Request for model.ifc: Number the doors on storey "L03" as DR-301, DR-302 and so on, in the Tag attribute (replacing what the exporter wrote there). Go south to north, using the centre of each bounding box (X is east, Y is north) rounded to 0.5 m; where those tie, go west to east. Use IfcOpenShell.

First a look at what the model holds.

```python
import ifcopenshell
import ifcopenshell.util.element
import ifcopenshell.util.placement

model = ifcopenshell.open("model.ifc")
print(model.schema)
storey = next(s for s in model.by_type("IfcBuildingStorey") if s.Name == "L03")
doors = [e for e in ifcopenshell.util.element.get_decomposition(storey) if e.is_a("IfcDoor")]
for e in sorted(doors, key=lambda e: e.id()):
    origin = ifcopenshell.util.placement.get_local_placement(e.ObjectPlacement)[:3, 3]
    print(e.id(), e.Tag, e.Name, origin.round(2) + 0.0, sep=" | ")
```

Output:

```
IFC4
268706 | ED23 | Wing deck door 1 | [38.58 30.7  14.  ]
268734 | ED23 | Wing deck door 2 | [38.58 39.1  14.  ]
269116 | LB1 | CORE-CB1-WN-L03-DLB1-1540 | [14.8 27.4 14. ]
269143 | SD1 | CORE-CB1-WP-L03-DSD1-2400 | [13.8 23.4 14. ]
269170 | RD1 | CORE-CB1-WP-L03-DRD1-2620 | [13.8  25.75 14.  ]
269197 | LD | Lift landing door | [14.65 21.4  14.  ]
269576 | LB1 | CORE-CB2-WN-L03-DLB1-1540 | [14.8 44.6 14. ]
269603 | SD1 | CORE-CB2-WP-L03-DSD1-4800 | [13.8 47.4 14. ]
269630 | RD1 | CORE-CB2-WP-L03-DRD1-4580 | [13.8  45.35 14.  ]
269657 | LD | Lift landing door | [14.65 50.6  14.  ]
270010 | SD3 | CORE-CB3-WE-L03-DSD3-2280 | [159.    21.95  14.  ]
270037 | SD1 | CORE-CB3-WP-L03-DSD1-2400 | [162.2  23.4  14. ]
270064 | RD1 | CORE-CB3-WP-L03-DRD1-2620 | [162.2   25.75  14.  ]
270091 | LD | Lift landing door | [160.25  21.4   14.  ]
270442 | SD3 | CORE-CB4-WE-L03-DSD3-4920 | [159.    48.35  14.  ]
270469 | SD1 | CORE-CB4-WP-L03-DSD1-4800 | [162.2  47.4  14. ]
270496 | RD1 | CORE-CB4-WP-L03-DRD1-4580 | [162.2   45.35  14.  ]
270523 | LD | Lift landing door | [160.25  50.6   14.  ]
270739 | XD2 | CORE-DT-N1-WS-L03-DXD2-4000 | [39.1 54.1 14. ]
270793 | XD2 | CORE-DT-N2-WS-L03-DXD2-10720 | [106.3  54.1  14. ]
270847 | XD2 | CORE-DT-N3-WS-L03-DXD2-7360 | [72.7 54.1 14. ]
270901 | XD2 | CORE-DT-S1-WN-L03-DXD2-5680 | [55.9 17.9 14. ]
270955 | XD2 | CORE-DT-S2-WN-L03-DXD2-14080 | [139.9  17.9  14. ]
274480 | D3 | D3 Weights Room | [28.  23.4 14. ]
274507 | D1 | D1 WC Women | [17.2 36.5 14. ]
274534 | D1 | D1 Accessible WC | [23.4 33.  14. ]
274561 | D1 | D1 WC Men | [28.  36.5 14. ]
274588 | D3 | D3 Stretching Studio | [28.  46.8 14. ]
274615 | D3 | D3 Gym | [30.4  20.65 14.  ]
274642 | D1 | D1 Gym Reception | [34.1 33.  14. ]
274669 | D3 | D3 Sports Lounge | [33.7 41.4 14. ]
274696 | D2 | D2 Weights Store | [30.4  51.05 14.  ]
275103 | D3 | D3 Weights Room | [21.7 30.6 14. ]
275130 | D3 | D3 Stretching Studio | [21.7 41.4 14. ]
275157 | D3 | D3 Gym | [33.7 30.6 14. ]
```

```python
import ifcopenshell
import ifcopenshell.geom
import ifcopenshell.util.element
import ifcopenshell.util.shape

model = ifcopenshell.open("model.ifc")
settings = ifcopenshell.geom.settings()
settings.set("use-world-coords", True)


def centre(element):
    shape = ifcopenshell.geom.create_shape(settings, element)
    return ifcopenshell.util.shape.get_bbox_centroid(shape.geometry)


storey = next(s for s in model.by_type("IfcBuildingStorey") if s.Name == "L03")
doors = [e for e in ifcopenshell.util.element.get_decomposition(storey) if e.is_a("IfcDoor")]

# Insertion points can sit at a corner or the storey origin, so sort by the geometry (in metres).
centres = {e: centre(e) for e in doors}
doors.sort(key=lambda e: (round(centres[e][1] / 0.5), centres[e][0]))

for i, e in enumerate(doors, start=1):
    number = f"DR-3{i:02d}"
    e.Tag = number
    print(e.id(), number)

model.write("model_updated.ifc")
```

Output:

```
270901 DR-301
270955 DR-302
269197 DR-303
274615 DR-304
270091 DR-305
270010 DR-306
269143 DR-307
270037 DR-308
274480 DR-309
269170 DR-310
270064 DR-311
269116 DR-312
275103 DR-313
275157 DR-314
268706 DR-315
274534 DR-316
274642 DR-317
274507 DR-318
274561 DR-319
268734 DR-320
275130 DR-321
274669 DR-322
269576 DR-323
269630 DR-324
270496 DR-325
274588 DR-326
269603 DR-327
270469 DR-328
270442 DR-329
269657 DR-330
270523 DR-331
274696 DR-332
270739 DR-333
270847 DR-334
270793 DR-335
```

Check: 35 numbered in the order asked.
